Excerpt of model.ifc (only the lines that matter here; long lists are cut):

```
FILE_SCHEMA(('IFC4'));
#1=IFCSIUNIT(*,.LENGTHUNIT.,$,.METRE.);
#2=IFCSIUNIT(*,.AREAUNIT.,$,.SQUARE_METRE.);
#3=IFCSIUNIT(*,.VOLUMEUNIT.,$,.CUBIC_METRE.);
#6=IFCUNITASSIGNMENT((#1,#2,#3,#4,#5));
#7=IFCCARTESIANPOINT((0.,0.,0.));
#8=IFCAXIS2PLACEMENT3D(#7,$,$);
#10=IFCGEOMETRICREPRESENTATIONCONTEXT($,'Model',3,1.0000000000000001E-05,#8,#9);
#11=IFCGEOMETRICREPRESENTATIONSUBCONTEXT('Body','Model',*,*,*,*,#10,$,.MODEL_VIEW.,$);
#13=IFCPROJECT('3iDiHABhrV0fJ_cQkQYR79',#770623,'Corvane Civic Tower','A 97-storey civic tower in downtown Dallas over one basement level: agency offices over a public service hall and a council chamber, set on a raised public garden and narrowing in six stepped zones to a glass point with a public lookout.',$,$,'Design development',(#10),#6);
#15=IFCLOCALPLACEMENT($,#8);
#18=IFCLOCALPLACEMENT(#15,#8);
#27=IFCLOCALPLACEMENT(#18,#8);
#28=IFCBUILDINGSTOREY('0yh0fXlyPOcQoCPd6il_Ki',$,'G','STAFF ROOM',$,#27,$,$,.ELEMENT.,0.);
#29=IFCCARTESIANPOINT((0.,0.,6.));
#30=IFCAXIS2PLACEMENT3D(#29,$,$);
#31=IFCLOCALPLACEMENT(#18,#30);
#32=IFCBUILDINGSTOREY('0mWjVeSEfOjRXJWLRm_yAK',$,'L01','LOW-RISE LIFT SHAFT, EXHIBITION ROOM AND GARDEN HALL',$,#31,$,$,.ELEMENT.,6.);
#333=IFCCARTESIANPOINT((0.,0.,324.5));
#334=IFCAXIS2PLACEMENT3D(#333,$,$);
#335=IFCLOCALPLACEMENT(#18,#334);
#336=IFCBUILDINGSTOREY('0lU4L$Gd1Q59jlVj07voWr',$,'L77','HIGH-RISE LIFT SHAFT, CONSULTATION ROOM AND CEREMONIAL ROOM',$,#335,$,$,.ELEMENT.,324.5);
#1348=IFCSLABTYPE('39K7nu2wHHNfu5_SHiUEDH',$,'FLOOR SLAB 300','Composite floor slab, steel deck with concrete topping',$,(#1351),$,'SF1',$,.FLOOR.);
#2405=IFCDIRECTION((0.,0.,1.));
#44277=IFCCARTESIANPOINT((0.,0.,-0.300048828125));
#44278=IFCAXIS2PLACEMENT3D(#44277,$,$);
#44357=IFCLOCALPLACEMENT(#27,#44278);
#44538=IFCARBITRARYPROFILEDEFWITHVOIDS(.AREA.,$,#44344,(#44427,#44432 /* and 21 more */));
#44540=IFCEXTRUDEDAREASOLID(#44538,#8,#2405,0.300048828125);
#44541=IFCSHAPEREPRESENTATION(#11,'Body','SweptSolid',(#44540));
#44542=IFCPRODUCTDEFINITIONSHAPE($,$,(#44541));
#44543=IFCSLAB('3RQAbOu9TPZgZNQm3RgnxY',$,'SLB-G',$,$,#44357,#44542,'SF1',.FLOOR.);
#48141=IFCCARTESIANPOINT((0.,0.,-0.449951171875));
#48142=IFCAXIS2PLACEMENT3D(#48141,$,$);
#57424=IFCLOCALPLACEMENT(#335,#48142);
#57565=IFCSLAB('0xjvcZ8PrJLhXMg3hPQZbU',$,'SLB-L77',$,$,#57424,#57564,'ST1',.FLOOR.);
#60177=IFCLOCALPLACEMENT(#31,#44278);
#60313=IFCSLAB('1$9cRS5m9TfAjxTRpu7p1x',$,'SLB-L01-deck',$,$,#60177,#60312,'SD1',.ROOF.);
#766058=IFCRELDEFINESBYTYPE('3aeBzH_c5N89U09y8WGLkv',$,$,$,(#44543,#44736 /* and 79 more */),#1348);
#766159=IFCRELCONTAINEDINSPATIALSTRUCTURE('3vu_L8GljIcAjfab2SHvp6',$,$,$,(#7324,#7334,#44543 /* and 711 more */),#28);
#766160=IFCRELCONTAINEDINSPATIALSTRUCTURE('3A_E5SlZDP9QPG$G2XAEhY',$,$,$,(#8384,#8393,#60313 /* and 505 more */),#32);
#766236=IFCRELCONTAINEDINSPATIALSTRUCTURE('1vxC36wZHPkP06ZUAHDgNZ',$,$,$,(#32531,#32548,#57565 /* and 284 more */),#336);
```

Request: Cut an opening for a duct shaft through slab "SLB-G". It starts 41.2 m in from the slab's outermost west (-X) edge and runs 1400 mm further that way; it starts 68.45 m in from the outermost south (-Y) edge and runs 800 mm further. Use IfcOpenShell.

```python
import numpy as np
import ifcopenshell
import ifcopenshell.api.feature
import ifcopenshell.api.geometry
import ifcopenshell.api.root
import ifcopenshell.geom
import ifcopenshell.util.placement
import ifcopenshell.util.representation
import ifcopenshell.util.shape
import ifcopenshell.util.unit

model = ifcopenshell.open("model.ifc")
unit_scale = ifcopenshell.util.unit.calculate_unit_scale(model)
settings = ifcopenshell.geom.settings()


def volume(element):
    """Net volume in cubic metres, openings subtracted."""
    shape = ifcopenshell.geom.create_shape(settings, element)
    return ifcopenshell.util.shape.get_volume(shape.geometry)


slab = model.by_guid("3RQAbOu9TPZgZNQm3RgnxY")
before = volume(slab)

# Extent in the slab's own axes, in metres. The edges named are its -X and -Y sides.
slab_shape = ifcopenshell.geom.create_shape(settings, slab)
vertices = ifcopenshell.util.shape.get_vertices(slab_shape.geometry)
x_min, y_min, bottom = vertices.min(axis=0)
top = vertices[:, 2].max()

opening = ifcopenshell.api.root.create_entity(model, ifc_class="IfcOpeningElement", name="Duct shaft opening", predefined_type="OPENING")
context = ifcopenshell.util.representation.get_context(model, "Model", "Body", "MODEL_VIEW")
width, depth = 1.4, 0.8
outline = [(0.0, 0.0), (width, 0.0), (width, depth), (0.0, depth), (0.0, 0.0)]
# Overshoot both faces by 50 mm so the cut is clean.
shape = ifcopenshell.api.geometry.add_slab_representation(
    model, context=context, depth=top - bottom + 0.1, polyline=outline
)
ifcopenshell.api.geometry.assign_representation(model, product=opening, representation=shape)

matrix = ifcopenshell.util.placement.get_local_placement(slab.ObjectPlacement)
matrix[:, 3] = matrix @ np.append(np.array([x_min + 41.2, y_min + 68.45, bottom - 0.05]) / unit_scale, 1.0)
ifcopenshell.api.geometry.edit_object_placement(model, product=opening, matrix=matrix, is_si=False)
ifcopenshell.api.feature.add_feature(model, feature=opening, element=slab)

after = volume(slab)

print(f"slab volume {before:.3f} -> {after:.3f} m3")

model.write("model_edited.ifc")
```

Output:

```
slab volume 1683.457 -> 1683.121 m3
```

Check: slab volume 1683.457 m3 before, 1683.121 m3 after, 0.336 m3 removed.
